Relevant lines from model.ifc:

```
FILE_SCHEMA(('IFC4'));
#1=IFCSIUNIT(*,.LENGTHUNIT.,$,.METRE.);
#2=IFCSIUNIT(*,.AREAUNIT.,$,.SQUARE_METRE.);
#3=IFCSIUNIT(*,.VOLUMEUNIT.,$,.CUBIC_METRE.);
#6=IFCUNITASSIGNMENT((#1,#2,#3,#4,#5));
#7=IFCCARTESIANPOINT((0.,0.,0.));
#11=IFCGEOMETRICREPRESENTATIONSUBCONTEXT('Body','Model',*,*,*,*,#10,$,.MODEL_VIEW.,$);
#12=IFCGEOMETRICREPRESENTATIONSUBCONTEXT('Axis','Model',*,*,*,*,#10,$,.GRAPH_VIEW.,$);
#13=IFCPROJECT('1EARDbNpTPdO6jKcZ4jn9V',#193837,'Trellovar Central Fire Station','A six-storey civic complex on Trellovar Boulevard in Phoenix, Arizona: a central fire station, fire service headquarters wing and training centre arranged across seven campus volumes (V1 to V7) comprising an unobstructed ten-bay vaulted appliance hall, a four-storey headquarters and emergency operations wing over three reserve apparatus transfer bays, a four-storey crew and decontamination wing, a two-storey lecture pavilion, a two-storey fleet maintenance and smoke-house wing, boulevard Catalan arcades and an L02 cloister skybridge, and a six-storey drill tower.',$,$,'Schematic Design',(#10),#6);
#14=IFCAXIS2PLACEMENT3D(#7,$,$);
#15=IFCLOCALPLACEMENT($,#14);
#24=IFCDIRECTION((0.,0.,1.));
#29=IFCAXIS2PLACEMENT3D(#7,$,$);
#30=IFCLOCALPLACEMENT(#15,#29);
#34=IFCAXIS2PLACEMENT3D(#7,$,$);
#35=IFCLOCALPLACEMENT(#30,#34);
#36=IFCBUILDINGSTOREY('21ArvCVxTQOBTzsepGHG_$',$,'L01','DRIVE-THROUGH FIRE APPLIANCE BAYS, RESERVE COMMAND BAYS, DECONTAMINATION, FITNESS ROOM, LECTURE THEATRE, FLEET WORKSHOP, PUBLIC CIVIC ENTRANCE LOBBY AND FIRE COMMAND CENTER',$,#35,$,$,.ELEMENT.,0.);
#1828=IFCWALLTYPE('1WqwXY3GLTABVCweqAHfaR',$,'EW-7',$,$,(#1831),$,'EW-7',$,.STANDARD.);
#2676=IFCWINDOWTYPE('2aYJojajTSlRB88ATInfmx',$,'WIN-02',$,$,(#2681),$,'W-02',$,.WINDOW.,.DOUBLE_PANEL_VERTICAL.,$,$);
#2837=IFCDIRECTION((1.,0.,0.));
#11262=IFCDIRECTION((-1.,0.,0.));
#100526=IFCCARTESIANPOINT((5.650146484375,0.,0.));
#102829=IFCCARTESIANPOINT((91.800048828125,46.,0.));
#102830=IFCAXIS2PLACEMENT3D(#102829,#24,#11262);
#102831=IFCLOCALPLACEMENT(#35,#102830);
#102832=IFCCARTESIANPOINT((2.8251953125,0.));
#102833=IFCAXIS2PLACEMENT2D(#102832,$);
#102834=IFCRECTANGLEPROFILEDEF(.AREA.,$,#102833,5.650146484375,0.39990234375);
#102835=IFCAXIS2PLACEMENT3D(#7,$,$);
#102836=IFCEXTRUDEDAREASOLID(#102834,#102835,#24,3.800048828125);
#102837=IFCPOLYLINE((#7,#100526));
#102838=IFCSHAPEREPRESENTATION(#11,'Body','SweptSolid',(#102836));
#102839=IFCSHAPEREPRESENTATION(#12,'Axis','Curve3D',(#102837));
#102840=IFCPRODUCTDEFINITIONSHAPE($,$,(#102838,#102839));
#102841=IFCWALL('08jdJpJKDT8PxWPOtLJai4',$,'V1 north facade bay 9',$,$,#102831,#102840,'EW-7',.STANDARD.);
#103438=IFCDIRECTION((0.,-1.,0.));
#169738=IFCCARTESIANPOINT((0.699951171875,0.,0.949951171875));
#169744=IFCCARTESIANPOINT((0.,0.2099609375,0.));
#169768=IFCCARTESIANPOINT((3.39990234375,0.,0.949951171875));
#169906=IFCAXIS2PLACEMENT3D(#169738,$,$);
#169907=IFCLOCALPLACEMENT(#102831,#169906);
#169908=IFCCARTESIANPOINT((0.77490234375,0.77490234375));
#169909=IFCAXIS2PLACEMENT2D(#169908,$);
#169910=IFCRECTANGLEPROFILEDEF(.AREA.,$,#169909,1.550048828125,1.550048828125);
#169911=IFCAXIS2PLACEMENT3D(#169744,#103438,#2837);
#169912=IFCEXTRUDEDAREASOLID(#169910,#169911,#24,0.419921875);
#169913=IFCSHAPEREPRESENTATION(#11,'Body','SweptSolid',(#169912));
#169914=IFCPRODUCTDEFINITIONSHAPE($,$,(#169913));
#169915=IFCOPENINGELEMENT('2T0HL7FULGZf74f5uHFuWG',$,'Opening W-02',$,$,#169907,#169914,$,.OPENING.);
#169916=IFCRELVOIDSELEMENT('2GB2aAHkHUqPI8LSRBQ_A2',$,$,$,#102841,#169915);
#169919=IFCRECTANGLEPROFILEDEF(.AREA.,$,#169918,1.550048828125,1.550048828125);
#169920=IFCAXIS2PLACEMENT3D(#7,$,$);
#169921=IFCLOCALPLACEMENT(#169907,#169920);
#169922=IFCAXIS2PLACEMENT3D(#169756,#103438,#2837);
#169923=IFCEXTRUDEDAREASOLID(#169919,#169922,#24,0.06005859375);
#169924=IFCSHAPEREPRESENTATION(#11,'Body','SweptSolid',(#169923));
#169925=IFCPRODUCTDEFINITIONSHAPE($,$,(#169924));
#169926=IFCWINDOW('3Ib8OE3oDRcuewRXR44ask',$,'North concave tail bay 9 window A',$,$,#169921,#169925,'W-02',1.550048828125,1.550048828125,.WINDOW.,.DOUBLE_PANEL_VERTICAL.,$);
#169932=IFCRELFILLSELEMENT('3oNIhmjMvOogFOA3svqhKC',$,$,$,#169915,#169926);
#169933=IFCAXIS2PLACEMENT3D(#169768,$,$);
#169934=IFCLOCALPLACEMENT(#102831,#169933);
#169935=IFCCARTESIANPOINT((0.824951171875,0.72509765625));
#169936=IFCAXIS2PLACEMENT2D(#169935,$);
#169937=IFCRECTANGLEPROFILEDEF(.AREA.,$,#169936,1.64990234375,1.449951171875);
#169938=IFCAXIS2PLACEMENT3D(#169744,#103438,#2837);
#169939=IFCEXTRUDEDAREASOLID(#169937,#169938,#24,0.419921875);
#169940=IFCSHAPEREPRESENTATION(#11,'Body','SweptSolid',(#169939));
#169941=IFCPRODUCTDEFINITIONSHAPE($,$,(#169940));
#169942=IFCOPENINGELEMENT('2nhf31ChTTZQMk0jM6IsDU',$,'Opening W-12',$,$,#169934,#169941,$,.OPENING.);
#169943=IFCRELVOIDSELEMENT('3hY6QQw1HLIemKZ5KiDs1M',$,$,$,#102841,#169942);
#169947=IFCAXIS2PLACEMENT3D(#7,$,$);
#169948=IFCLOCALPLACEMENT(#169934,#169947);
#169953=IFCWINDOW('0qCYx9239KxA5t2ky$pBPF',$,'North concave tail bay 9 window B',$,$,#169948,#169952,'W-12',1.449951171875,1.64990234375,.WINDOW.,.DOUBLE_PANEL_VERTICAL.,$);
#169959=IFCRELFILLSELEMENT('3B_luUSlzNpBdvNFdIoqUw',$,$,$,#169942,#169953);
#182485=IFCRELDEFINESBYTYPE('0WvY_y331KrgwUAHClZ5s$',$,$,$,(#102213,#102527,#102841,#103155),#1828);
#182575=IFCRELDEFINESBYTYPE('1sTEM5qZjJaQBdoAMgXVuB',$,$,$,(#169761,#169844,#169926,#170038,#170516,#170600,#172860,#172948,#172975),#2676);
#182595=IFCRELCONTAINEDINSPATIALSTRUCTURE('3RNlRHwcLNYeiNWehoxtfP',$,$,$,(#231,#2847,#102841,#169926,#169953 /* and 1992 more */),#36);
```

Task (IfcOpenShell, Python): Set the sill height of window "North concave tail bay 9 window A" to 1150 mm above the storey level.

```python
import numpy as np
import ifcopenshell
import ifcopenshell.api.geometry
import ifcopenshell.geom
import ifcopenshell.util.element
import ifcopenshell.util.placement
import ifcopenshell.util.shape
import ifcopenshell.util.unit

model = ifcopenshell.open("model.ifc")
unit_scale = ifcopenshell.util.unit.calculate_unit_scale(model)

window = model.by_guid("3Ib8OE3oDRcuewRXR44ask")
opening = window.FillsVoids[0].RelatingOpeningElement
storey = ifcopenshell.util.element.get_container(window, ifc_class="IfcBuildingStorey")
level = ifcopenshell.util.placement.get_local_placement(storey.ObjectPlacement)[2, 3]

# The opening's origin need not be at the sill, so measure its lowest point.
shape = ifcopenshell.geom.create_shape(ifcopenshell.geom.settings(), opening)
bottom = ifcopenshell.util.shape.get_shape_bottom_elevation(shape, shape.geometry) / unit_scale
dz = level + 1.15 - bottom

shift = np.array([0.0, 0.0, dz])
# The window is placed relative to its opening, so it follows when the opening moves.
matrix = ifcopenshell.util.placement.get_local_placement(opening.ObjectPlacement)
matrix[:3, 3] += shift
ifcopenshell.api.geometry.edit_object_placement(
    model, product=opening, matrix=matrix, is_si=False, should_transform_children=True
)

print(f"moved by {dz * unit_scale:+.3f} m")

model.write("model-out.ifc")
```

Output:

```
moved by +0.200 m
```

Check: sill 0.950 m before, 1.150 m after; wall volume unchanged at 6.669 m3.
